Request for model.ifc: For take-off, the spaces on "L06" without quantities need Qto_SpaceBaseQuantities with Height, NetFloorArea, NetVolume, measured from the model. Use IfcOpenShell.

First a look at what the model holds.

```python
import ifcopenshell
import ifcopenshell.util.element
import ifcopenshell.util.unit

model = ifcopenshell.open("model.ifc")
print(model.schema)
for unit_type in ("LENGTHUNIT", "AREAUNIT", "VOLUMEUNIT"):
    print(unit_type, ifcopenshell.util.unit.calculate_unit_scale(model, unit_type))
storey = next(s for s in model.by_type("IfcBuildingStorey") if s.Name == "L06")
spaces = [e for e in ifcopenshell.util.element.get_decomposition(storey) if e.is_a("IfcSpace")]
for e in sorted(spaces, key=lambda e: e.id()):
    print(e.id(), e.is_a(), e.Name, list(ifcopenshell.util.element.get_psets(e, qtos_only=True)), sep=" | ")
```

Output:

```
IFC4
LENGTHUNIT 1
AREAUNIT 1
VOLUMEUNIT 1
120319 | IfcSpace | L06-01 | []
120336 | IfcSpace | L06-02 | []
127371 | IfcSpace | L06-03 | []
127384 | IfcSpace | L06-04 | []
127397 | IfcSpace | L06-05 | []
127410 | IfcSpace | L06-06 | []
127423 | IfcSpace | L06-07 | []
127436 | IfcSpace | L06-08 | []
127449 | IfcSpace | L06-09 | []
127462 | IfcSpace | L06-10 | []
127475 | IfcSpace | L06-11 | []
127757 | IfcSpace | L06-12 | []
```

```python
import ifcopenshell
import ifcopenshell.api.pset
import ifcopenshell.geom
import ifcopenshell.util.element
import ifcopenshell.util.shape
import ifcopenshell.util.unit

model = ifcopenshell.open("model.ifc")
unit_scale = ifcopenshell.util.unit.calculate_unit_scale(model)
area_scale = ifcopenshell.util.unit.calculate_unit_scale(model, "AREAUNIT")
volume_scale = ifcopenshell.util.unit.calculate_unit_scale(model, "VOLUMEUNIT")
settings = ifcopenshell.geom.settings()

storey = next(s for s in model.by_type("IfcBuildingStorey") if s.Name == "L06")
spaces = [e for e in ifcopenshell.util.element.get_decomposition(storey) if e.is_a("IfcSpace")]

for e in sorted(spaces, key=lambda e: e.id()):
    if ifcopenshell.util.element.get_psets(e, qtos_only=True, should_inherit=False):
        continue
    # Geometry comes back in metres, in the element's own axes.
    shape = ifcopenshell.geom.create_shape(settings, e)
    values = {
        "Height": ifcopenshell.util.shape.get_z(shape.geometry) / unit_scale,
        "NetFloorArea": ifcopenshell.util.shape.get_footprint_area(shape.geometry) / area_scale,
        "NetVolume": ifcopenshell.util.shape.get_volume(shape.geometry) / volume_scale,
    }
    qto = ifcopenshell.api.pset.add_qto(model, product=e, name="Qto_SpaceBaseQuantities")
    ifcopenshell.api.pset.edit_qto(model, qto=qto, properties=values)
    print(e.id(), {k: round(v, 3) for k, v in values.items()})

model.write("model_v2.ifc")
```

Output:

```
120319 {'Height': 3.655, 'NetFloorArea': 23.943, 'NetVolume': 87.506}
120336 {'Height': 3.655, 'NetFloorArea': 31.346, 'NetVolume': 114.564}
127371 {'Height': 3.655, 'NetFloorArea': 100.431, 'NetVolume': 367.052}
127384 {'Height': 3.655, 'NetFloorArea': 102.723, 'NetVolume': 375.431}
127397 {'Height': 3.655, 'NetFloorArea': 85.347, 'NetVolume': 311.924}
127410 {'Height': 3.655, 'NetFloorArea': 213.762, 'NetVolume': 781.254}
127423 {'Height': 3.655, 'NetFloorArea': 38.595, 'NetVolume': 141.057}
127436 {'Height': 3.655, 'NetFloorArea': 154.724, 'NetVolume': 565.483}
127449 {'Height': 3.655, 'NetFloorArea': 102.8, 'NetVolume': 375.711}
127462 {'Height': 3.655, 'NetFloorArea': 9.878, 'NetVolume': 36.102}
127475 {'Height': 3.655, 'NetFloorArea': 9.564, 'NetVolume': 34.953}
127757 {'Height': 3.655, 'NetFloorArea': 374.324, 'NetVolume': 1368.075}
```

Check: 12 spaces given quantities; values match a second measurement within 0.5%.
